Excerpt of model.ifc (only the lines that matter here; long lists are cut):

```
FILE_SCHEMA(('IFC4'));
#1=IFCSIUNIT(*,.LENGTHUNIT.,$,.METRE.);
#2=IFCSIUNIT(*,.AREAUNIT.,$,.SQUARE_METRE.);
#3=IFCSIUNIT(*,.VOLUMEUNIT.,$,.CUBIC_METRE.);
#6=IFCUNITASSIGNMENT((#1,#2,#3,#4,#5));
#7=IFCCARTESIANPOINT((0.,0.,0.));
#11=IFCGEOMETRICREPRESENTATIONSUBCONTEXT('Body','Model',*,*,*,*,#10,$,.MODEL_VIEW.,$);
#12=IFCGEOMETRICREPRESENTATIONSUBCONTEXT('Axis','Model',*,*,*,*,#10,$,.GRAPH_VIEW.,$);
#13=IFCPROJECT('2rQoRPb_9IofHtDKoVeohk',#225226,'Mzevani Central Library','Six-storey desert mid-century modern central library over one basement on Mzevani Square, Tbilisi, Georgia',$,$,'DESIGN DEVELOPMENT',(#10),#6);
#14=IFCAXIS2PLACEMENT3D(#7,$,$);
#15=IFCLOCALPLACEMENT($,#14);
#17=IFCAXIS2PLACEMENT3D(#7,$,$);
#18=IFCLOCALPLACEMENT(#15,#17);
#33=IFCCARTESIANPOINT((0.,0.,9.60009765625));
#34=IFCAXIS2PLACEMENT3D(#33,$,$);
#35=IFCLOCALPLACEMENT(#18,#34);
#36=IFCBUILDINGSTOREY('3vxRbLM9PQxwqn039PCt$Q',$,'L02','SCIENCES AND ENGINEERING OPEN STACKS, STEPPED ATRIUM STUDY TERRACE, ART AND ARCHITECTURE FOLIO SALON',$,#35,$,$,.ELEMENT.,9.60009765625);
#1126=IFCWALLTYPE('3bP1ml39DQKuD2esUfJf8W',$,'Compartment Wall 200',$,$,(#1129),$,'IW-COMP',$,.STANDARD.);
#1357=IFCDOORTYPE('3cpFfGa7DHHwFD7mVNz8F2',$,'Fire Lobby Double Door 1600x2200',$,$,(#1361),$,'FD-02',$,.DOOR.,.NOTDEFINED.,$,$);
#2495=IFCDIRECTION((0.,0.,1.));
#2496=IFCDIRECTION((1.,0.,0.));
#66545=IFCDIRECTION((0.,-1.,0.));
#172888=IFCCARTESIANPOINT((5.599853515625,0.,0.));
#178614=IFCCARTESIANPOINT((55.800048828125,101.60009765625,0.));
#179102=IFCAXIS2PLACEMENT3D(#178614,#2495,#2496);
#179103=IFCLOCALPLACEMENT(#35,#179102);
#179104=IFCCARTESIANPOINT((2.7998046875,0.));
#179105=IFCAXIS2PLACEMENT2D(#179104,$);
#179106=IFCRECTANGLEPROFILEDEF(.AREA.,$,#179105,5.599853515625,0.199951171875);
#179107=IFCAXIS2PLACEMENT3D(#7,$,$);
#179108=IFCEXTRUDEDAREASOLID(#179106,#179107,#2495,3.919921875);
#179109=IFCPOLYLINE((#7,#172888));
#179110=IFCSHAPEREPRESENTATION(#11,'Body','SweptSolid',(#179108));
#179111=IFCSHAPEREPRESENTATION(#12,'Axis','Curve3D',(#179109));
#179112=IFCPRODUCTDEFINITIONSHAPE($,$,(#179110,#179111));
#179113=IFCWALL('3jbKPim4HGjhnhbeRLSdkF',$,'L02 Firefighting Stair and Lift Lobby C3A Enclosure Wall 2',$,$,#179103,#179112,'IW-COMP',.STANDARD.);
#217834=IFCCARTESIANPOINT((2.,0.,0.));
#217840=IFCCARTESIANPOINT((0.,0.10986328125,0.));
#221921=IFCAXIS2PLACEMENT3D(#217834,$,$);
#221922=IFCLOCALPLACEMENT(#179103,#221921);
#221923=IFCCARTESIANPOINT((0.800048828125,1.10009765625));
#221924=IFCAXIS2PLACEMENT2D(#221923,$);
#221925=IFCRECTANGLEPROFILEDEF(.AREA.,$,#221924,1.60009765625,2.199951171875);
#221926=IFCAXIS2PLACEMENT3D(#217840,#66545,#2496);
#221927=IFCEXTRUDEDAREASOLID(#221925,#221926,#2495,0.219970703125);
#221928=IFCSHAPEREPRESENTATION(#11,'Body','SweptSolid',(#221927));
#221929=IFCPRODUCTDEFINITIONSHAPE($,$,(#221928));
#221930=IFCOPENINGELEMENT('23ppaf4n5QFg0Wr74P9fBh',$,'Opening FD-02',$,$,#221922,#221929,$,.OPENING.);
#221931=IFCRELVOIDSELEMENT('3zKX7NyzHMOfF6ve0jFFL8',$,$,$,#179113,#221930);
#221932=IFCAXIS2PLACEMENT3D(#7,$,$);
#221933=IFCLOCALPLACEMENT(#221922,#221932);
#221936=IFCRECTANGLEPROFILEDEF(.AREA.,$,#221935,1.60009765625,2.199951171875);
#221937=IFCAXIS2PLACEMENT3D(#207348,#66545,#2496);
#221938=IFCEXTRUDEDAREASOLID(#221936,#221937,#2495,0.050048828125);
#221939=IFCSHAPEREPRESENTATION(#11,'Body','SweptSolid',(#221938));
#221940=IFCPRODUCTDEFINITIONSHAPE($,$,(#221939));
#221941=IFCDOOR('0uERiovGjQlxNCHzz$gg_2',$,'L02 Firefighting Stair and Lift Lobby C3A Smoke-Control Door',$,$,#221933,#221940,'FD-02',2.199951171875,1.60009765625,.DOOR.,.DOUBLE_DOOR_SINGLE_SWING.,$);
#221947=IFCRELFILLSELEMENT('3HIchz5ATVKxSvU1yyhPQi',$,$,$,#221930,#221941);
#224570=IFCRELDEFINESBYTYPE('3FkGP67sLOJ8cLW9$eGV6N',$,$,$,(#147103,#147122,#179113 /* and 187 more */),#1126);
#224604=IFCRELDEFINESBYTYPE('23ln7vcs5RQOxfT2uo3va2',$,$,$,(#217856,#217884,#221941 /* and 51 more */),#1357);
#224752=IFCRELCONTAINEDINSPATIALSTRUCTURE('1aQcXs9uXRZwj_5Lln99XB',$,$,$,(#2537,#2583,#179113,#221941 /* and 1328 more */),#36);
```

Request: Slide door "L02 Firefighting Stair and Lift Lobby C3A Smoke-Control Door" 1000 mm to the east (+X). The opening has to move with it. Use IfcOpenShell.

```python
import ifcopenshell
import ifcopenshell.api.geometry
import ifcopenshell.util.placement
import ifcopenshell.util.unit

model = ifcopenshell.open("model.ifc")
unit_scale = ifcopenshell.util.unit.calculate_unit_scale(model)

door = model.by_guid("0uERiovGjQlxNCHzz$gg_2")
opening = door.FillsVoids[0].RelatingOpeningElement
wall = opening.VoidsElements[0].RelatingBuildingElement

wall_matrix = ifcopenshell.util.placement.get_local_placement(wall.ObjectPlacement)
shift = wall_matrix[:3, 0] * 1 / unit_scale
before = ifcopenshell.util.placement.get_local_placement(door.ObjectPlacement)[:3, 3].copy()

# The door is placed relative to its opening, so it follows when the opening moves.
matrix = ifcopenshell.util.placement.get_local_placement(opening.ObjectPlacement)
matrix[:3, 3] += shift
ifcopenshell.api.geometry.edit_object_placement(
    model, product=opening, matrix=matrix, is_si=False, should_transform_children=True
)

after = ifcopenshell.util.placement.get_local_placement(door.ObjectPlacement)[:3, 3]
print("door moved by", (after - before).round(3) + 0.0)

model.write("model_updated.ifc")
```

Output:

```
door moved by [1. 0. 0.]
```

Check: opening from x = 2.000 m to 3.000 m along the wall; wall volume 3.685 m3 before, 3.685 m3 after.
